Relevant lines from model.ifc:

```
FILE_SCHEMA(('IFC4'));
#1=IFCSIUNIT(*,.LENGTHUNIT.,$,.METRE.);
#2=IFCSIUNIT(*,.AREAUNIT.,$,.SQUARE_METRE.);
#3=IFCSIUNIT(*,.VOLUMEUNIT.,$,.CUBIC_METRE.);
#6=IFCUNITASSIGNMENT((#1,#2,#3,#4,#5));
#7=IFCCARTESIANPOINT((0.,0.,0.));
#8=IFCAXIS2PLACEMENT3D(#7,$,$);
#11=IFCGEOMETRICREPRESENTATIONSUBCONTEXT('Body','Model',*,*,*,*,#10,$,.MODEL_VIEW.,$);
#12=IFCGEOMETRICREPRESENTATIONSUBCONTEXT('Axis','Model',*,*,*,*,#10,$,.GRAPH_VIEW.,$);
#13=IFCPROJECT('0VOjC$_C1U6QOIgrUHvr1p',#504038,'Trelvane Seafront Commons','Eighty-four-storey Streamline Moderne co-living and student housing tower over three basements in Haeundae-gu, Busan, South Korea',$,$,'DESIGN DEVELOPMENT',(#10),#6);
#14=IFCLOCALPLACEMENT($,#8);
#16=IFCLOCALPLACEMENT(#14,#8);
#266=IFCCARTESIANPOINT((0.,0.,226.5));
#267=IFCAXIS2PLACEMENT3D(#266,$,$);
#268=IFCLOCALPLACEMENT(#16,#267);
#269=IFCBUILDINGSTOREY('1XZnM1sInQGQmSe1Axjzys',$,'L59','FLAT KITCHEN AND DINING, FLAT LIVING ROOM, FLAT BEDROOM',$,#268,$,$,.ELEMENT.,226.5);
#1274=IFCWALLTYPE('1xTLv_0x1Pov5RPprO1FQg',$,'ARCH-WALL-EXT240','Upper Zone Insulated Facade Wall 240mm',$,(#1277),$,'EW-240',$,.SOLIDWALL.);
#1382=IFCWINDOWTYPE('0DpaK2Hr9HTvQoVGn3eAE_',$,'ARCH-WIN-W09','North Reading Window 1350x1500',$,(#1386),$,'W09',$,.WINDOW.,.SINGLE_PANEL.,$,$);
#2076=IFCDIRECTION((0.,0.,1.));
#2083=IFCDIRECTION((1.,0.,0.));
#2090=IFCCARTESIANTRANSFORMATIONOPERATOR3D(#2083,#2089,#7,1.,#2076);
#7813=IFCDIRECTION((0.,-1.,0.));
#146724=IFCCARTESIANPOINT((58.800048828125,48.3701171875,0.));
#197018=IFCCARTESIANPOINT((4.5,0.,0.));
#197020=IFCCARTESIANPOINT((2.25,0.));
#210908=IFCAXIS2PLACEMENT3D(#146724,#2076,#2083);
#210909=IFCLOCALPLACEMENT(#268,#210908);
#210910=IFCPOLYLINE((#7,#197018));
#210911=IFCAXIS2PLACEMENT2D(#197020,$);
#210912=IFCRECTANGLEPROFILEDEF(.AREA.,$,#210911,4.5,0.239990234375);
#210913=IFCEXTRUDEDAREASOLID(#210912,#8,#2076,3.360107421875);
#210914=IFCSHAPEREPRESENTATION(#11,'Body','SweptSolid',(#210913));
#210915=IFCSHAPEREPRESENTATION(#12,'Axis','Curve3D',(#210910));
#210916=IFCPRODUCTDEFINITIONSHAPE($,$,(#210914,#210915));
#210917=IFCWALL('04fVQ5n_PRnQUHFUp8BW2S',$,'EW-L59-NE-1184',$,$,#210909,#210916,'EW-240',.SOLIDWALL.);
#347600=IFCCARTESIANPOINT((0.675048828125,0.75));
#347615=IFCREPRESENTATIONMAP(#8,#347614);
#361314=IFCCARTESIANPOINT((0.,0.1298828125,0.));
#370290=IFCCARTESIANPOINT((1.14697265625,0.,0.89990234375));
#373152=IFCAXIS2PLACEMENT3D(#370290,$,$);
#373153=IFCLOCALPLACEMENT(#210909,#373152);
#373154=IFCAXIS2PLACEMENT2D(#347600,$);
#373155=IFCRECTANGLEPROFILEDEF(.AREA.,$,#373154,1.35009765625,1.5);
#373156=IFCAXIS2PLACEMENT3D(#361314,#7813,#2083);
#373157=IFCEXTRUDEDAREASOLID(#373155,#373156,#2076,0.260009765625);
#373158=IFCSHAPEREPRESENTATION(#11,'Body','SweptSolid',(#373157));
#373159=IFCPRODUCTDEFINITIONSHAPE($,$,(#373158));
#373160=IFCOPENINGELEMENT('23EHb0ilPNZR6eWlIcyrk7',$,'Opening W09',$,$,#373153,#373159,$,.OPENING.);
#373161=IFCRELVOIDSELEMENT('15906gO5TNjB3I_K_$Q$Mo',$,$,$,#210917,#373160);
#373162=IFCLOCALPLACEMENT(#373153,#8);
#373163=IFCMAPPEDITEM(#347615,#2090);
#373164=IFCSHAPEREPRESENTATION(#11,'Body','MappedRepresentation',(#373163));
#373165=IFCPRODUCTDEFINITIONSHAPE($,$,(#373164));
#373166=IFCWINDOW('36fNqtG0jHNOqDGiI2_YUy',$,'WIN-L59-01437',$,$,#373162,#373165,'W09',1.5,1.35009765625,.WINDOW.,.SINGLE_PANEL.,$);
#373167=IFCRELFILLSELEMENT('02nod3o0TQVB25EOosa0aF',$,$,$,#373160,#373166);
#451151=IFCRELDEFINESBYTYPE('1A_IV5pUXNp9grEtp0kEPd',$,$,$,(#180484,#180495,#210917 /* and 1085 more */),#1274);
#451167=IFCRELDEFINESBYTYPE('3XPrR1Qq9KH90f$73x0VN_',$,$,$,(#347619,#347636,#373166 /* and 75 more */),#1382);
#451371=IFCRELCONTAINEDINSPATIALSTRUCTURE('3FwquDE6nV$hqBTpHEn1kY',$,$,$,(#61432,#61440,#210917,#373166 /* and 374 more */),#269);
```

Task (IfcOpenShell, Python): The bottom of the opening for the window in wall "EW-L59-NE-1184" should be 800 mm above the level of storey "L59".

```python
import numpy as np
import ifcopenshell
import ifcopenshell.api.geometry
import ifcopenshell.geom
import ifcopenshell.util.element
import ifcopenshell.util.placement
import ifcopenshell.util.shape
import ifcopenshell.util.unit

model = ifcopenshell.open("model.ifc")
unit_scale = ifcopenshell.util.unit.calculate_unit_scale(model)

window = model.by_guid("36fNqtG0jHNOqDGiI2_YUy")
opening = window.FillsVoids[0].RelatingOpeningElement
storey = ifcopenshell.util.element.get_container(window, ifc_class="IfcBuildingStorey")
level = ifcopenshell.util.placement.get_local_placement(storey.ObjectPlacement)[2, 3]

# The opening's origin need not be at the sill, so measure its lowest point.
shape = ifcopenshell.geom.create_shape(ifcopenshell.geom.settings(), opening)
bottom = ifcopenshell.util.shape.get_shape_bottom_elevation(shape, shape.geometry) / unit_scale
dz = level + 0.8 / unit_scale - bottom

shift = np.array([0.0, 0.0, dz])
# The window is placed relative to its opening, so it follows when the opening moves.
matrix = ifcopenshell.util.placement.get_local_placement(opening.ObjectPlacement)
matrix[:3, 3] += shift
ifcopenshell.api.geometry.edit_object_placement(
    model, product=opening, matrix=matrix, is_si=False, should_transform_children=True
)

print(f"moved by {dz * unit_scale:+.3f} m")

model.write("model-out.ifc")
```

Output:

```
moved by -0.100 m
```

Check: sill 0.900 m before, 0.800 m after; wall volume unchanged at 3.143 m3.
